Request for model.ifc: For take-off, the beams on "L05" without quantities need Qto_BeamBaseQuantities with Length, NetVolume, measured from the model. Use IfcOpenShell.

First a look at what the model holds.

```python
import ifcopenshell
import ifcopenshell.util.element
import ifcopenshell.util.unit

model = ifcopenshell.open("model.ifc")
print(model.schema)
for unit_type in ("LENGTHUNIT", "AREAUNIT", "VOLUMEUNIT"):
    print(unit_type, ifcopenshell.util.unit.calculate_unit_scale(model, unit_type))
storey = next(s for s in model.by_type("IfcBuildingStorey") if s.Name == "L05")
beams = [e for e in ifcopenshell.util.element.get_decomposition(storey) if e.is_a("IfcBeam")]
for e in sorted(beams, key=lambda e: e.id()):
    print(e.id(), e.is_a(), e.Name, list(ifcopenshell.util.element.get_psets(e, qtos_only=True)), sep=" | ")
```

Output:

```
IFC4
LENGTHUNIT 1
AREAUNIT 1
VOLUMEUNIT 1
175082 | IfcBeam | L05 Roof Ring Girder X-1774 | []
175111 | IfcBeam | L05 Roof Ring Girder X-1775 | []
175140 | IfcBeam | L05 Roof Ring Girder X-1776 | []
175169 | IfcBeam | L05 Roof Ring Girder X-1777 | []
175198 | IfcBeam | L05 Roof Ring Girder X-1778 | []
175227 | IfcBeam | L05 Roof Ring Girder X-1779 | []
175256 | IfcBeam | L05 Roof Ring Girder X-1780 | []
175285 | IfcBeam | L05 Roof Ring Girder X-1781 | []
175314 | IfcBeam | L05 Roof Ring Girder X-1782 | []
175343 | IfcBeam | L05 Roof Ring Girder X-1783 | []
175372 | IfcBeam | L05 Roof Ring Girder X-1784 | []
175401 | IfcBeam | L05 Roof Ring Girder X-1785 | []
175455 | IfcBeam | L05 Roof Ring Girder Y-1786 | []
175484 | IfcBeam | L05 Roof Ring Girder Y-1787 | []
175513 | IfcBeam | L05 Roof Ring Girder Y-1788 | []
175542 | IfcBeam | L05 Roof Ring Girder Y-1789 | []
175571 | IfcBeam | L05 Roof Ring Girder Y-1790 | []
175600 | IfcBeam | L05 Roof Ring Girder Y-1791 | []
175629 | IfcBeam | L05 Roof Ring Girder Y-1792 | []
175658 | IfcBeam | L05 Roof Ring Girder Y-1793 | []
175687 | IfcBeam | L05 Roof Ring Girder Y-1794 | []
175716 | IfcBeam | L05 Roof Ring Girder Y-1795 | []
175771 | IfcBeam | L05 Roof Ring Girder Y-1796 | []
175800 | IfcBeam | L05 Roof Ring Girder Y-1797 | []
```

```python
import ifcopenshell
import ifcopenshell.api.pset
import ifcopenshell.geom
import ifcopenshell.util.element
import ifcopenshell.util.shape
import ifcopenshell.util.unit

model = ifcopenshell.open("model.ifc")
unit_scale = ifcopenshell.util.unit.calculate_unit_scale(model)
volume_scale = ifcopenshell.util.unit.calculate_unit_scale(model, "VOLUMEUNIT")
settings = ifcopenshell.geom.settings()

storey = next(s for s in model.by_type("IfcBuildingStorey") if s.Name == "L05")
beams = [e for e in ifcopenshell.util.element.get_decomposition(storey) if e.is_a("IfcBeam")]

for e in sorted(beams, key=lambda e: e.id()):
    if ifcopenshell.util.element.get_psets(e, qtos_only=True, should_inherit=False):
        continue
    # Geometry comes back in metres, in the element's own axes.
    shape = ifcopenshell.geom.create_shape(settings, e)
    values = {
        "Length": ifcopenshell.util.shape.get_max_xyz(shape.geometry) / unit_scale,
        "NetVolume": ifcopenshell.util.shape.get_volume(shape.geometry) / volume_scale,
    }
    qto = ifcopenshell.api.pset.add_qto(model, product=e, name="Qto_BeamBaseQuantities")
    ifcopenshell.api.pset.edit_qto(model, qto=qto, properties=values)
    print(e.id(), {k: round(v, 3) for k, v in values.items()})

model.write("model-out.ifc")
```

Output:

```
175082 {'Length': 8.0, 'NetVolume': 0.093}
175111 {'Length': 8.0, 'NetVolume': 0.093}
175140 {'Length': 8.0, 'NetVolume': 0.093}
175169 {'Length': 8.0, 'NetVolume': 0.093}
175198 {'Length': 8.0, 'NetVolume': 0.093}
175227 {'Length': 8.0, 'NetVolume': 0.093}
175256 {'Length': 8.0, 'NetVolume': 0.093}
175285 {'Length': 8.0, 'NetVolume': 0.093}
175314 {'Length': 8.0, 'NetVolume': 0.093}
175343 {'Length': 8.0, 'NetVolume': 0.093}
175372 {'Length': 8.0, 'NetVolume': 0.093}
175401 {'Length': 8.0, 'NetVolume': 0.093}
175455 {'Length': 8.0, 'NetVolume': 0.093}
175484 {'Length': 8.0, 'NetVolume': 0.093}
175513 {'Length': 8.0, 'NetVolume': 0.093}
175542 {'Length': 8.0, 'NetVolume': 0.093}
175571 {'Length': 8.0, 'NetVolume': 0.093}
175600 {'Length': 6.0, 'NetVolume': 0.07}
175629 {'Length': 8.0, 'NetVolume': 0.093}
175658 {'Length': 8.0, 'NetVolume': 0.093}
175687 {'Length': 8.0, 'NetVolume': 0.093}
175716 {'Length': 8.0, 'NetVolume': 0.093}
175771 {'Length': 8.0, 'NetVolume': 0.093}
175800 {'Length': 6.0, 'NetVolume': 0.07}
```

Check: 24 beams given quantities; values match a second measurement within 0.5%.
